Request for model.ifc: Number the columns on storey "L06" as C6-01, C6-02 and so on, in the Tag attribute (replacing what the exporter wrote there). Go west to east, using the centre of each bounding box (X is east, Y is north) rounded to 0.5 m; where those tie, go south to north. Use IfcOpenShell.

First a look at what the model holds.

```python
import ifcopenshell
import ifcopenshell.util.element
import ifcopenshell.util.placement

model = ifcopenshell.open("model.ifc")
print(model.schema)
storey = next(s for s in model.by_type("IfcBuildingStorey") if s.Name == "L06")
columns = [e for e in ifcopenshell.util.element.get_decomposition(storey) if e.is_a("IfcColumn")]
for e in sorted(columns, key=lambda e: e.id()):
    origin = ifcopenshell.util.placement.get_local_placement(e.ObjectPlacement)[:3, 3]
    print(e.id(), e.Tag, e.Name, origin.round(2) + 0.0, sep=" | ")
```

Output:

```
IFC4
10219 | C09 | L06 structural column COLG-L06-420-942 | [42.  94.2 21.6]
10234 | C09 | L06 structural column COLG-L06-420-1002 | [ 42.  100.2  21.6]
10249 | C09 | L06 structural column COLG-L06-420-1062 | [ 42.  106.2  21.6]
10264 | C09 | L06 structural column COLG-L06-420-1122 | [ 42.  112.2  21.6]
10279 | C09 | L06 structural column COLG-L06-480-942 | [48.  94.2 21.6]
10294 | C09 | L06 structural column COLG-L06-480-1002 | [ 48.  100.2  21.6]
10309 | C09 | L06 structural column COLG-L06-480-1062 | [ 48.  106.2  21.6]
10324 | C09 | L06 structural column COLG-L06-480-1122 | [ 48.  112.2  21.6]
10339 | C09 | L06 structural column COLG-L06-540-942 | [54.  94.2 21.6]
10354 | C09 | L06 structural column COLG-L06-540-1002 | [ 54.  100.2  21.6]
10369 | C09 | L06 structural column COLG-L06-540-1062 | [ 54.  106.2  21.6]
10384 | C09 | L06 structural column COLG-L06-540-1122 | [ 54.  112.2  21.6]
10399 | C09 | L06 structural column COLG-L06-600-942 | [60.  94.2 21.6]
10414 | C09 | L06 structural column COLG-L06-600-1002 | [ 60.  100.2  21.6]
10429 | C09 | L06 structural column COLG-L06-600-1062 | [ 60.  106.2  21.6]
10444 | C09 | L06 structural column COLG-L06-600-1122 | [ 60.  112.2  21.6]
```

```python
import ifcopenshell
import ifcopenshell.geom
import ifcopenshell.util.element
import ifcopenshell.util.shape

model = ifcopenshell.open("model.ifc")
settings = ifcopenshell.geom.settings()
settings.set("use-world-coords", True)


def centre(element):
    shape = ifcopenshell.geom.create_shape(settings, element)
    return ifcopenshell.util.shape.get_bbox_centroid(shape.geometry)


storey = next(s for s in model.by_type("IfcBuildingStorey") if s.Name == "L06")
columns = [e for e in ifcopenshell.util.element.get_decomposition(storey) if e.is_a("IfcColumn")]

# Insertion points can sit at a corner or the storey origin, so sort by the geometry (in metres).
centres = {e: centre(e) for e in columns}
columns.sort(key=lambda e: (round(centres[e][0] / 0.5), centres[e][1]))

for i, e in enumerate(columns, start=1):
    number = f"C6-{i:02d}"
    e.Tag = number
    print(e.id(), number)

model.write("model_updated.ifc")
```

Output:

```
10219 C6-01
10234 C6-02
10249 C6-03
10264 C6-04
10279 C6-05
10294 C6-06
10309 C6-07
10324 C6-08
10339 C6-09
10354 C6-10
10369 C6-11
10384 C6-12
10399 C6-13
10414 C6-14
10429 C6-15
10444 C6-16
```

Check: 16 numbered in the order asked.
